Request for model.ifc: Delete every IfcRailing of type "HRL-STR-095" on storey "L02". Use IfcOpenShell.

First a look at what the model holds.

```python
import ifcopenshell
import ifcopenshell.util.element

model = ifcopenshell.open("model.ifc")
print(model.schema)
storey = next(s for s in model.by_type("IfcBuildingStorey") if s.Name == "L02")
railings = [e for e in ifcopenshell.util.element.get_decomposition(storey) if e.is_a("IfcRailing")]
seen = {}
for e in railings:
    element_type = ifcopenshell.util.element.get_type(e)
    name = element_type.Name if element_type not in (None, e) else None
    seen[name] = seen.get(name, 0) + 1
for name, count in sorted(seen.items(), key=str):
    print(count, "x", name)
```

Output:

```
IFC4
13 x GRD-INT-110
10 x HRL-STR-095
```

```python
import ifcopenshell
import ifcopenshell.api.root
import ifcopenshell.util.element

model = ifcopenshell.open("model.ifc")

storey = next(s for s in model.by_type("IfcBuildingStorey") if s.Name == "L02")
railings = [e for e in ifcopenshell.util.element.get_decomposition(storey) if e.is_a("IfcRailing")]
targets = [e for e in railings if (t := ifcopenshell.util.element.get_type(e)) not in (None, e) and t.Name == "HRL-STR-095"]

for e in targets:
    ifcopenshell.api.root.remove_product(model, product=e)
print(len(targets), "removed")

model.write("model_edited.ifc")
```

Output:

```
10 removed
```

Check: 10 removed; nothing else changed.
